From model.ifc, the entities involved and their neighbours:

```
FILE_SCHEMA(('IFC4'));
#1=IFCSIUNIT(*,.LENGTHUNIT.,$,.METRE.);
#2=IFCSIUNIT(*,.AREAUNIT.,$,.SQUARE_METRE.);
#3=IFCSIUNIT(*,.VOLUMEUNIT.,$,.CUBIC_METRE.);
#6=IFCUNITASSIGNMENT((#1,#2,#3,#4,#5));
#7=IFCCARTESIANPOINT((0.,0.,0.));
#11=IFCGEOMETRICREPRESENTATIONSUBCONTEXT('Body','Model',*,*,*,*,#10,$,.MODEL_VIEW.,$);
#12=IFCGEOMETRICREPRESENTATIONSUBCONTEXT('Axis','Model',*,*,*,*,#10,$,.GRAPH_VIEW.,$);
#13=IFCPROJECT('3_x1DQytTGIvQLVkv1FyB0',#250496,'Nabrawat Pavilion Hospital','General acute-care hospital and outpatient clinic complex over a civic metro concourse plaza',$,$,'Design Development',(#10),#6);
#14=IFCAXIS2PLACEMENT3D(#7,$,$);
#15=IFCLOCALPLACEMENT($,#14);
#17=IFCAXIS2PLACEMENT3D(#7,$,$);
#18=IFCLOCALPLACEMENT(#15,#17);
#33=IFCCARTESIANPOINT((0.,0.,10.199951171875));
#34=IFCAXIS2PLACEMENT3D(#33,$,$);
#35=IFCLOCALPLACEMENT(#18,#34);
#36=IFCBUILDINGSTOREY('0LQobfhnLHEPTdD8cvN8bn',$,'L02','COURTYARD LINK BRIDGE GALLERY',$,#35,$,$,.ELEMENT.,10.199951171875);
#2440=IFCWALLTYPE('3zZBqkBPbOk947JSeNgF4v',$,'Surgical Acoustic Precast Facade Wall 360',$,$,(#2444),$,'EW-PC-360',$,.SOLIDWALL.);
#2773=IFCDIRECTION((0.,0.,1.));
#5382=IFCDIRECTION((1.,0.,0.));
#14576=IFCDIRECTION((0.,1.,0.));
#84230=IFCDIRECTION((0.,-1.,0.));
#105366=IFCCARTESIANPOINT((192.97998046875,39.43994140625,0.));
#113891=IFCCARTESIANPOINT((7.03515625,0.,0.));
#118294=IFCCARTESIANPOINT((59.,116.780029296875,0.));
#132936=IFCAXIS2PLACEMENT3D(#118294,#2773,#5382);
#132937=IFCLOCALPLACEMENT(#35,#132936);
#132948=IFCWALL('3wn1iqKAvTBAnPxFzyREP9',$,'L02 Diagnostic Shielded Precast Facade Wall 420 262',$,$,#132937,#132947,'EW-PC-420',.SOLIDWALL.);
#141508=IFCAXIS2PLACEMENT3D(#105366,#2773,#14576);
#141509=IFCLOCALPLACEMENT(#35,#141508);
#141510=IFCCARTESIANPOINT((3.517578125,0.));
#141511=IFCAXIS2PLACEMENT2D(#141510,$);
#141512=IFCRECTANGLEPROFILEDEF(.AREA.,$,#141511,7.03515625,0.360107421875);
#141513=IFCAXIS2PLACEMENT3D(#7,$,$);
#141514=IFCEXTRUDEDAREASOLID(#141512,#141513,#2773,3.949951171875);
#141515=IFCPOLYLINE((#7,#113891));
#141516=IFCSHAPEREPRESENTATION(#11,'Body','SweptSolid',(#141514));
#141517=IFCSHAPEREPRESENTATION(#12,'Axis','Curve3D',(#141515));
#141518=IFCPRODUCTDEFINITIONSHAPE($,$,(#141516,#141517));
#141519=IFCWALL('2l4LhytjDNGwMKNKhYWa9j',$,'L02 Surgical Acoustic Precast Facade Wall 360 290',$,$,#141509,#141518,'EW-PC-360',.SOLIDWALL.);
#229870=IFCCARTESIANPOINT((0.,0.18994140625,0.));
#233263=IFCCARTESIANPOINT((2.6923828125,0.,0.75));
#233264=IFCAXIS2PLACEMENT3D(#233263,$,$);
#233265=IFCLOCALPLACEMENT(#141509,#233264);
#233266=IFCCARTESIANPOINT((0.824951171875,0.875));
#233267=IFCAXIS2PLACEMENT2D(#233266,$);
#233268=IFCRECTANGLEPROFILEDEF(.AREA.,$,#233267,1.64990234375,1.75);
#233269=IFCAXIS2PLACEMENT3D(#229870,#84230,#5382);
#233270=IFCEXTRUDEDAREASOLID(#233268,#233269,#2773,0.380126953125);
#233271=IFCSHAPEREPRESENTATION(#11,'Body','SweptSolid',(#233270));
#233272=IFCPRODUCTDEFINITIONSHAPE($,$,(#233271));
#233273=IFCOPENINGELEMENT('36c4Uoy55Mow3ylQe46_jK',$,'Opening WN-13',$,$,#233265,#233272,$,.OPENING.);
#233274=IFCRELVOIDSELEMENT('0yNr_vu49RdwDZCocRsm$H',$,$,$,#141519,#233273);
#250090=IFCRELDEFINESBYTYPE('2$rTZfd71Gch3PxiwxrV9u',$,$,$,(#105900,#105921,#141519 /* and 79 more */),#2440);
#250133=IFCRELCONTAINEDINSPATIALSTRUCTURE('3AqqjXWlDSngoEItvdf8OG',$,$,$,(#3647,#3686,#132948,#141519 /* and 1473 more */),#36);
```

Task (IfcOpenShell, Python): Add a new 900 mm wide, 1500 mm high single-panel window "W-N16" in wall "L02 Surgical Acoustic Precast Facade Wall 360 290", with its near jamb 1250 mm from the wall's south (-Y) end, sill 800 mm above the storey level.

```python
import numpy as np
import ifcopenshell
import ifcopenshell.api.feature
import ifcopenshell.api.geometry
import ifcopenshell.api.root
import ifcopenshell.api.spatial
import ifcopenshell.geom
import ifcopenshell.util.element
import ifcopenshell.util.placement
import ifcopenshell.util.representation
import ifcopenshell.util.shape
import ifcopenshell.util.unit

model = ifcopenshell.open("model.ifc")
unit_scale = ifcopenshell.util.unit.calculate_unit_scale(model)
settings = ifcopenshell.geom.settings()


def volume(element):
    """Net volume in cubic metres, openings subtracted."""
    shape = ifcopenshell.geom.create_shape(settings, element)
    return ifcopenshell.util.shape.get_volume(shape.geometry)


wall = model.by_id(141519)
storey = ifcopenshell.util.element.get_container(wall, ifc_class="IfcBuildingStorey")
context = ifcopenshell.util.representation.get_context(model, "Model", "Body", "MODEL_VIEW")
before = volume(wall)

width, height, from_end, sill = 0.9, 1.5, 1.25, 0.8  # metres

# The wall runs along its own X axis, and the end named is its -X end.
wall_shape = ifcopenshell.geom.create_shape(settings, wall)
x, y, z = ifcopenshell.util.shape.get_vertices(wall_shape.geometry).T
start = x.min() + from_end
face, thickness = float(y.min()), float(y.max() - y.min())
wall_matrix = ifcopenshell.util.placement.get_local_placement(wall.ObjectPlacement)
level = ifcopenshell.util.placement.get_local_placement(storey.ObjectPlacement)[2, 3]


def in_wall(x, y):
    """Placement at x, y metres in the wall's axes, at sill height."""
    matrix = wall_matrix.copy()
    matrix[:, 3] = wall_matrix @ np.array([x / unit_scale, y / unit_scale, 0.0, 1.0])
    matrix[2, 3] = level + sill / unit_scale
    return matrix


# Opening: a box that overshoots both wall faces by 50 mm.
opening = ifcopenshell.api.root.create_entity(model, ifc_class="IfcOpeningElement", predefined_type="OPENING")
box = ifcopenshell.api.geometry.add_wall_representation(
    model, context=context, length=width, height=height, thickness=thickness + 0.1
)
ifcopenshell.api.geometry.assign_representation(model, product=opening, representation=box)
ifcopenshell.api.geometry.edit_object_placement(model, product=opening, matrix=in_wall(start, face - 0.05), is_si=False)
ifcopenshell.api.feature.add_feature(model, feature=opening, element=wall)

window = ifcopenshell.api.root.create_entity(model, ifc_class="IfcWindow", name="W-N16", predefined_type="WINDOW")
window.OverallWidth, window.OverallHeight = width / unit_scale, height / unit_scale
window.PartitioningType = "SINGLE_PANEL"
body = ifcopenshell.api.geometry.add_window_representation(
    model,
    context=context,
    overall_width=window.OverallWidth,
    overall_height=window.OverallHeight,
    partition_type="SINGLE_PANEL",
)
ifcopenshell.api.geometry.assign_representation(model, product=window, representation=body)
ifcopenshell.api.spatial.assign_container(model, products=[window], relating_structure=storey)
ifcopenshell.api.feature.add_filling(model, opening=opening, element=window)

# Centre the window in the wall's thickness.
ifcopenshell.api.geometry.edit_object_placement(model, product=window, matrix=in_wall(start, face), is_si=False)
window_shape = ifcopenshell.geom.create_shape(settings, window)
depth = ifcopenshell.util.shape.get_vertices(window_shape.geometry)[:, 1]
offset = face + thickness / 2 - (depth.min() + depth.max()) / 2
ifcopenshell.api.geometry.edit_object_placement(model, product=window, matrix=in_wall(start, offset), is_si=False)

after = volume(wall)

print(f"wall volume {before:.3f} -> {after:.3f} m3")

model.write("model_rev.ifc")
```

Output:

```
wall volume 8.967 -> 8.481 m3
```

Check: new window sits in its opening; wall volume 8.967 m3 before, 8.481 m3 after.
